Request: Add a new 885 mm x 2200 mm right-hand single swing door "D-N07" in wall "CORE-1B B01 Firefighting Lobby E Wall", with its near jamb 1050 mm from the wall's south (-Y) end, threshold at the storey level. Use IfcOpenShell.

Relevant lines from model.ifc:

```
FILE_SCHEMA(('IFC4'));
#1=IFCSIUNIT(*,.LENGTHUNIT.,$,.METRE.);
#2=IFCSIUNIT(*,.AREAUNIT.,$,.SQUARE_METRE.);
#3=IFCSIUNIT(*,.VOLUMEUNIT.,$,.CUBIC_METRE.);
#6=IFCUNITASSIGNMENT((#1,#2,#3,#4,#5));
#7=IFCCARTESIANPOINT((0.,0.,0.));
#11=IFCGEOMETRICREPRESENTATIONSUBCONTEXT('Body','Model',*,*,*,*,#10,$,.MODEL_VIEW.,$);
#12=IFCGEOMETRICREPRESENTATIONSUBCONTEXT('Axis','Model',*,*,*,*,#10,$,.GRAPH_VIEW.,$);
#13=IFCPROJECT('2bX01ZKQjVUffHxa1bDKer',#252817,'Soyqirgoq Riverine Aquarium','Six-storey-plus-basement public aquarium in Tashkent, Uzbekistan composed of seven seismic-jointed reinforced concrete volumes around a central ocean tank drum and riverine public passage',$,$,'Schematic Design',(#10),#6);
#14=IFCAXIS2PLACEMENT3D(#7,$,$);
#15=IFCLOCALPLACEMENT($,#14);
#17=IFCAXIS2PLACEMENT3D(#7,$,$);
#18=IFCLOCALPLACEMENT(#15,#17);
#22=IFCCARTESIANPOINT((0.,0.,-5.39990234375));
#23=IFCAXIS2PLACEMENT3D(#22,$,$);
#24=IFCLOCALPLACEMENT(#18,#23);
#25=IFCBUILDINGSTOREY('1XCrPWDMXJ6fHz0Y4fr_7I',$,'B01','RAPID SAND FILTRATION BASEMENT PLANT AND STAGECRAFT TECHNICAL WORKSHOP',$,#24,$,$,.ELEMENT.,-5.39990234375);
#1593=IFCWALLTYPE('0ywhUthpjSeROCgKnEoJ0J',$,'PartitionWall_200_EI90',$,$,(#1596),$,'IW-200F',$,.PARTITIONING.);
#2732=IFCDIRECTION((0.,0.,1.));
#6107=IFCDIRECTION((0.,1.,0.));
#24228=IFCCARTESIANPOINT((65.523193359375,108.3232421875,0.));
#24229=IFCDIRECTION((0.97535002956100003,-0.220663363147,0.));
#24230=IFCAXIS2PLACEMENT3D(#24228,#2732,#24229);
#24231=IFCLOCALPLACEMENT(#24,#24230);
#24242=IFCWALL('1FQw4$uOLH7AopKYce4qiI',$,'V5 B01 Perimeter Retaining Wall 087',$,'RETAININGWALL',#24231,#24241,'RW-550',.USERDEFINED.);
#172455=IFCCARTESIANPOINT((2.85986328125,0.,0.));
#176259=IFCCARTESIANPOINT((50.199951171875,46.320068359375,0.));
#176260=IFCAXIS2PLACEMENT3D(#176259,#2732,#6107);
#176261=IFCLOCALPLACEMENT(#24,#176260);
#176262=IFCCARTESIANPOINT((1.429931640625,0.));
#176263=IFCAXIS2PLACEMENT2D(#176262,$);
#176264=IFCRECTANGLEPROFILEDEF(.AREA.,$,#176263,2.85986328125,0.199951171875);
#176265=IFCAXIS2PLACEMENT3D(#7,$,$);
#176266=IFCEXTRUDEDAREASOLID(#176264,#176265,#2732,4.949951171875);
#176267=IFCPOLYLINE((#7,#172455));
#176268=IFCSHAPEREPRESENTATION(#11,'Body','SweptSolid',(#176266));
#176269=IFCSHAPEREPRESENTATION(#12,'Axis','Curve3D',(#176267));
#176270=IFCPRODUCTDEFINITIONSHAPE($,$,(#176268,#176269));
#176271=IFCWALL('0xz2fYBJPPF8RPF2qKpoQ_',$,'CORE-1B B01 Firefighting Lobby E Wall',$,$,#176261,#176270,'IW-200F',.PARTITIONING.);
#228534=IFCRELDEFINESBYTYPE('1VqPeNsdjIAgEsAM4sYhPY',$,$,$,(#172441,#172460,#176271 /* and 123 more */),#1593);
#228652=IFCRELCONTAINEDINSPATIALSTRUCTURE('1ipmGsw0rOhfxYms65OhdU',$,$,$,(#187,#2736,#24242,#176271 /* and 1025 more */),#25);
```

```python
import numpy as np
import ifcopenshell
import ifcopenshell.api.feature
import ifcopenshell.api.geometry
import ifcopenshell.api.root
import ifcopenshell.api.spatial
import ifcopenshell.geom
import ifcopenshell.util.element
import ifcopenshell.util.placement
import ifcopenshell.util.representation
import ifcopenshell.util.shape
import ifcopenshell.util.unit

model = ifcopenshell.open("model.ifc")
unit_scale = ifcopenshell.util.unit.calculate_unit_scale(model)
settings = ifcopenshell.geom.settings()


def volume(element):
    """Net volume in cubic metres, openings subtracted."""
    shape = ifcopenshell.geom.create_shape(settings, element)
    return ifcopenshell.util.shape.get_volume(shape.geometry)


wall = model.by_id(176271)
storey = ifcopenshell.util.element.get_container(wall, ifc_class="IfcBuildingStorey")
context = ifcopenshell.util.representation.get_context(model, "Model", "Body", "MODEL_VIEW")
before = volume(wall)

width, height, from_end, sill = 0.885, 2.2, 1.05, 0.0  # metres

# The wall runs along its own X axis, and the end named is its -X end.
wall_shape = ifcopenshell.geom.create_shape(settings, wall)
x, y, z = ifcopenshell.util.shape.get_vertices(wall_shape.geometry).T
start = x.min() + from_end
face, thickness = float(y.min()), float(y.max() - y.min())
wall_matrix = ifcopenshell.util.placement.get_local_placement(wall.ObjectPlacement)
level = ifcopenshell.util.placement.get_local_placement(storey.ObjectPlacement)[2, 3]


def in_wall(x, y):
    """Placement at x, y metres in the wall's axes, at sill height."""
    matrix = wall_matrix.copy()
    matrix[:, 3] = wall_matrix @ np.array([x / unit_scale, y / unit_scale, 0.0, 1.0])
    matrix[2, 3] = level + sill / unit_scale
    return matrix


# Opening: a box that overshoots both wall faces by 50 mm.
opening = ifcopenshell.api.root.create_entity(model, ifc_class="IfcOpeningElement", predefined_type="OPENING")
box = ifcopenshell.api.geometry.add_wall_representation(
    model, context=context, length=width, height=height, thickness=thickness + 0.1
)
ifcopenshell.api.geometry.assign_representation(model, product=opening, representation=box)
ifcopenshell.api.geometry.edit_object_placement(model, product=opening, matrix=in_wall(start, face - 0.05), is_si=False)
ifcopenshell.api.feature.add_feature(model, feature=opening, element=wall)

door = ifcopenshell.api.root.create_entity(model, ifc_class="IfcDoor", name="D-N07", predefined_type="DOOR")
door.OverallWidth, door.OverallHeight = width / unit_scale, height / unit_scale
door.OperationType = "SINGLE_SWING_RIGHT"
body = ifcopenshell.api.geometry.add_door_representation(
    model,
    context=context,
    overall_width=door.OverallWidth,
    overall_height=door.OverallHeight,
    operation_type="SINGLE_SWING_RIGHT",
    lining_properties={"LiningDepth": thickness / unit_scale, "ThresholdDepth": thickness / unit_scale},
)
ifcopenshell.api.geometry.assign_representation(model, product=door, representation=body)
ifcopenshell.api.spatial.assign_container(model, products=[door], relating_structure=storey)
ifcopenshell.api.feature.add_filling(model, opening=opening, element=door)

# The lining spans the wall, so the door starts at the wall face.
ifcopenshell.api.geometry.edit_object_placement(model, product=door, matrix=in_wall(start, face), is_si=False)

after = volume(wall)

print(f"wall volume {before:.3f} -> {after:.3f} m3")

model.write("model_edited.ifc")
```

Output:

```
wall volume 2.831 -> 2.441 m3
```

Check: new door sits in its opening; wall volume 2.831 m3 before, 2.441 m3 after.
